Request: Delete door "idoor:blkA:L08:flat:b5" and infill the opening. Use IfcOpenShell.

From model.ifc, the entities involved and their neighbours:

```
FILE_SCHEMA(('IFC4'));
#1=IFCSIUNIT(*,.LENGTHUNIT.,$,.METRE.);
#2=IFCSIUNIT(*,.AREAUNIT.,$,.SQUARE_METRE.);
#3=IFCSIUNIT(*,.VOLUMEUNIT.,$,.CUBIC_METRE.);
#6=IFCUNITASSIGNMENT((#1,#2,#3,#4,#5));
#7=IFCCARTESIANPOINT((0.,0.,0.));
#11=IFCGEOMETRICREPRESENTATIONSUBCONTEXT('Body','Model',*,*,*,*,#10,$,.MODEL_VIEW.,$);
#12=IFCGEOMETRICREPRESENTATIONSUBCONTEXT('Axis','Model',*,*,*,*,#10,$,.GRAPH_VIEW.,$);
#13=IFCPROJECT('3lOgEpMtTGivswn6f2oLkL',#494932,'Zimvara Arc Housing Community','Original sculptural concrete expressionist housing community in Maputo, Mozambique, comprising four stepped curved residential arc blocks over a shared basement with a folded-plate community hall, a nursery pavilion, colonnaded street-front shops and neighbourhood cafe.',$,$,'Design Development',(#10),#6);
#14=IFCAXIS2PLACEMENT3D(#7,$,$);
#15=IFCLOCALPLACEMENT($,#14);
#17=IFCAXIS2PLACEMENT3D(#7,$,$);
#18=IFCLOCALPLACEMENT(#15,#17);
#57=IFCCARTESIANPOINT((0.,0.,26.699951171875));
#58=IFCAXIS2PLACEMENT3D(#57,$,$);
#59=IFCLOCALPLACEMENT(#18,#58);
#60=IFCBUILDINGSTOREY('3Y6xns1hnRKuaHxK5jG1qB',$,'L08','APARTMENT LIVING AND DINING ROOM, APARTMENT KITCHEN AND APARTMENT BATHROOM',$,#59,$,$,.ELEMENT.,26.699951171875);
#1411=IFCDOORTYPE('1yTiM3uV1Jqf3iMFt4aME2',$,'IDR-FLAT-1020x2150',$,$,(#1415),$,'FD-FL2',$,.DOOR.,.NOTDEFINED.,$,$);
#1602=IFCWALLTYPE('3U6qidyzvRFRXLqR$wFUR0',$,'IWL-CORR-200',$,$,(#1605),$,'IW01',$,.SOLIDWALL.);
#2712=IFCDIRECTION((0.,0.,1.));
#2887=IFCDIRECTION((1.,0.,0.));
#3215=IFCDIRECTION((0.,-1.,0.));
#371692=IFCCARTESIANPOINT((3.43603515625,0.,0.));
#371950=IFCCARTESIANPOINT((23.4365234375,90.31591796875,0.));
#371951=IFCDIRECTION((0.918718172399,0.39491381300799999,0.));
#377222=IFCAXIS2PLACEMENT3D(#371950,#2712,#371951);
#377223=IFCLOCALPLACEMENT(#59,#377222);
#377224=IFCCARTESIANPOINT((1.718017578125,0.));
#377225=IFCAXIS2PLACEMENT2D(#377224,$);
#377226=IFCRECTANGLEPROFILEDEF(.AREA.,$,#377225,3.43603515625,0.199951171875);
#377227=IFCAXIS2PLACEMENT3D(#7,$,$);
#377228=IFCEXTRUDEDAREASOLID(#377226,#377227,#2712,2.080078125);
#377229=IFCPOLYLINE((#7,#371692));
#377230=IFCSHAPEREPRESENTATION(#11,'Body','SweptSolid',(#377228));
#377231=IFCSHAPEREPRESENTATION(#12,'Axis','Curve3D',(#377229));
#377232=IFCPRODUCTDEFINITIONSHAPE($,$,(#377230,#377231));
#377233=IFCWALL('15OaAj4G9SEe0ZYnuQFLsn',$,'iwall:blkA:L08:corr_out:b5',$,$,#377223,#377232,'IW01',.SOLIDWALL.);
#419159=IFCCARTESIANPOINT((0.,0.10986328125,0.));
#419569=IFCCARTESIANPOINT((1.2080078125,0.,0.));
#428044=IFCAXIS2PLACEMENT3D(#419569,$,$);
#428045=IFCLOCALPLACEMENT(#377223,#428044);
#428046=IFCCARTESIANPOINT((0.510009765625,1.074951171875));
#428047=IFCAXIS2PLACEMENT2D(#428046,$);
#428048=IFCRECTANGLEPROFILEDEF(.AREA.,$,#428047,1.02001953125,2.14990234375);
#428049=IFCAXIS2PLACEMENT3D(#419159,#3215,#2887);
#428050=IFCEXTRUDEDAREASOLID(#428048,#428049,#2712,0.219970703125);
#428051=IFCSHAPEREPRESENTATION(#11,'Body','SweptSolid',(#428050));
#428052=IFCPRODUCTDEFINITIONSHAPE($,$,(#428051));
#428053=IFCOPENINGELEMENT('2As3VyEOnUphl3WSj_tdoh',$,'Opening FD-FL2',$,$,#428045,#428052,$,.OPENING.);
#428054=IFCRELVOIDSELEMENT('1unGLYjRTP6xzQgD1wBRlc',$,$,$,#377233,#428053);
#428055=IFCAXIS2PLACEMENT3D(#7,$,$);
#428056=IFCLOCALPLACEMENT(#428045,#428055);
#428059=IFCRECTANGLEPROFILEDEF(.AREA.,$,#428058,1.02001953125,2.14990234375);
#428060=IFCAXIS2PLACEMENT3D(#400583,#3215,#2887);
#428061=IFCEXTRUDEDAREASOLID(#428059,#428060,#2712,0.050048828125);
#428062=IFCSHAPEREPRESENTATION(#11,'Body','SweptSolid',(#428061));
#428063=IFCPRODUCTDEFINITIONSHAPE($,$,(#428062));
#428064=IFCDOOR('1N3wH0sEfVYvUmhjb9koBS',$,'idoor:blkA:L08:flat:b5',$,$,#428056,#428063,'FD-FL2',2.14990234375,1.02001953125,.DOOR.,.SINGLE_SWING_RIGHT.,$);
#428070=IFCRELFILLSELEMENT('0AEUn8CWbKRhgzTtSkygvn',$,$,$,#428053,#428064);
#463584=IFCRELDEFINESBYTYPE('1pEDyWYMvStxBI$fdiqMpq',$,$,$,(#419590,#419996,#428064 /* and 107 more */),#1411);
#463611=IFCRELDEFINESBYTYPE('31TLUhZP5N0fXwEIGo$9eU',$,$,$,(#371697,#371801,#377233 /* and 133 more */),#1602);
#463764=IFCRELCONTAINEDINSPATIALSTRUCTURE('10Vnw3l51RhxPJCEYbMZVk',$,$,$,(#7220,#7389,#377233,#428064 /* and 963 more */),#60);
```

```python
import ifcopenshell
import ifcopenshell.api.feature
import ifcopenshell.api.root
import ifcopenshell.geom
import ifcopenshell.util.shape

model = ifcopenshell.open("model.ifc")
settings = ifcopenshell.geom.settings()


def volume(element):
    """Net volume in cubic metres, openings subtracted."""
    shape = ifcopenshell.geom.create_shape(settings, element)
    return ifcopenshell.util.shape.get_volume(shape.geometry)


door = model.by_guid("1N3wH0sEfVYvUmhjb9koBS")
opening = door.FillsVoids[0].RelatingOpeningElement
wall = opening.VoidsElements[0].RelatingBuildingElement
before = volume(wall)

ifcopenshell.api.root.remove_product(model, product=door)
ifcopenshell.api.feature.remove_feature(model, feature=opening)

after = volume(wall)

print(f"wall volume {before:.3f} -> {after:.3f} m3")

model.write("model_v2.ifc")
```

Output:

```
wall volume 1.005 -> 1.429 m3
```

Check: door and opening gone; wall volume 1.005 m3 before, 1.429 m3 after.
